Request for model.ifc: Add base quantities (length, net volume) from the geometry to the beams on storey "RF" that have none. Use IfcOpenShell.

First a look at what the model holds.

```python
import ifcopenshell
import ifcopenshell.util.element
import ifcopenshell.util.unit

model = ifcopenshell.open("model.ifc")
print(model.schema)
for unit_type in ("LENGTHUNIT", "AREAUNIT", "VOLUMEUNIT"):
    print(unit_type, ifcopenshell.util.unit.calculate_unit_scale(model, unit_type))
storey = next(s for s in model.by_type("IfcBuildingStorey") if s.Name == "RF")
beams = [e for e in ifcopenshell.util.element.get_decomposition(storey) if e.is_a("IfcBeam")]
for e in sorted(beams, key=lambda e: e.id()):
    print(e.id(), e.is_a(), e.Name, list(ifcopenshell.util.element.get_psets(e, qtos_only=True)), sep=" | ")
```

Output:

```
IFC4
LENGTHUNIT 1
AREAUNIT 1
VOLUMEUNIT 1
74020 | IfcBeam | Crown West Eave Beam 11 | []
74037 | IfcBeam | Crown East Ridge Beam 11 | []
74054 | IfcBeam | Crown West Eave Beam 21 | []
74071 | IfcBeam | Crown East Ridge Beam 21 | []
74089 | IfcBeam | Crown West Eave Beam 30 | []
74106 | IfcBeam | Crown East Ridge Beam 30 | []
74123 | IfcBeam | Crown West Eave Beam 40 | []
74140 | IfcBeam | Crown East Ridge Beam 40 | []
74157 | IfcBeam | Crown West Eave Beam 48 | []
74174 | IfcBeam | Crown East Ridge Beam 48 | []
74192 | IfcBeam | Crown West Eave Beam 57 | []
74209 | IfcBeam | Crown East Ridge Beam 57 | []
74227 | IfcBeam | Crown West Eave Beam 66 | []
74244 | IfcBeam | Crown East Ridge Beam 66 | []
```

```python
import ifcopenshell
import ifcopenshell.api.pset
import ifcopenshell.geom
import ifcopenshell.util.element
import ifcopenshell.util.shape
import ifcopenshell.util.unit

model = ifcopenshell.open("model.ifc")
unit_scale = ifcopenshell.util.unit.calculate_unit_scale(model)
volume_scale = ifcopenshell.util.unit.calculate_unit_scale(model, "VOLUMEUNIT")
settings = ifcopenshell.geom.settings()

storey = next(s for s in model.by_type("IfcBuildingStorey") if s.Name == "RF")
beams = [e for e in ifcopenshell.util.element.get_decomposition(storey) if e.is_a("IfcBeam")]

for e in sorted(beams, key=lambda e: e.id()):
    if ifcopenshell.util.element.get_psets(e, qtos_only=True, should_inherit=False):
        continue
    # Geometry comes back in metres, in the element's own axes.
    shape = ifcopenshell.geom.create_shape(settings, e)
    values = {
        "Length": ifcopenshell.util.shape.get_max_xyz(shape.geometry) / unit_scale,
        "NetVolume": ifcopenshell.util.shape.get_volume(shape.geometry) / volume_scale,
    }
    qto = ifcopenshell.api.pset.add_qto(model, product=e, name="Qto_BeamBaseQuantities")
    ifcopenshell.api.pset.edit_qto(model, qto=qto, properties=values)
    print(e.id(), {k: round(v, 3) for k, v in values.items()})

model.write("model_edited.ifc")
```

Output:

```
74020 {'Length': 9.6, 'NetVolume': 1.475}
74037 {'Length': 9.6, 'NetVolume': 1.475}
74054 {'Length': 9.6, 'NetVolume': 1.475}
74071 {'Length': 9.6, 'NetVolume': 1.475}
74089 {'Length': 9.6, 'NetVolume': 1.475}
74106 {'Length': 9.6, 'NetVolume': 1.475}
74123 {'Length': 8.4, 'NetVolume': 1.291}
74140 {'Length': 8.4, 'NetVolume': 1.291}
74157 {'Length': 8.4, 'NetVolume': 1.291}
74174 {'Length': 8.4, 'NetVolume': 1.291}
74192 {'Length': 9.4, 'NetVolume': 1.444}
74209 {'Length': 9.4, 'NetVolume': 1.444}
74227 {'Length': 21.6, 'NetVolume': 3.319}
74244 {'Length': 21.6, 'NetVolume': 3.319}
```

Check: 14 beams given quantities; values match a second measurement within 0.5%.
